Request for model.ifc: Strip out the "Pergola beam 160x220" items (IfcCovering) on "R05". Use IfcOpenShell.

First a look at what the model holds.

```python
import ifcopenshell
import ifcopenshell.util.element

model = ifcopenshell.open("model.ifc")
print(model.schema)
storey = next(s for s in model.by_type("IfcBuildingStorey") if s.Name == "R05")
coverings = [e for e in ifcopenshell.util.element.get_decomposition(storey) if e.is_a("IfcCovering")]
seen = {}
for e in coverings:
    element_type = ifcopenshell.util.element.get_type(e)
    name = element_type.Name if element_type not in (None, e) else None
    seen[name] = seen.get(name, 0) + 1
for name, count in sorted(seen.items(), key=str):
    print(count, "x", name)
```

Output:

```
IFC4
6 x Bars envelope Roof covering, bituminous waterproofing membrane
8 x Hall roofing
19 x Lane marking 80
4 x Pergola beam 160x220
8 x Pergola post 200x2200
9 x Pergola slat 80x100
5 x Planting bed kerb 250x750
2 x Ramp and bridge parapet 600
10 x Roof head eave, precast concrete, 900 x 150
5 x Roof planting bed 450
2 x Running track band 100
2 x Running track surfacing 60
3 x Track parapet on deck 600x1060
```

```python
import ifcopenshell
import ifcopenshell.api.root
import ifcopenshell.util.element

model = ifcopenshell.open("model.ifc")

storey = next(s for s in model.by_type("IfcBuildingStorey") if s.Name == "R05")
coverings = [e for e in ifcopenshell.util.element.get_decomposition(storey) if e.is_a("IfcCovering")]
targets = [e for e in coverings if (t := ifcopenshell.util.element.get_type(e)) not in (None, e) and t.Name == "Pergola beam 160x220"]

for e in targets:
    ifcopenshell.api.root.remove_product(model, product=e)
print(len(targets), "removed")

model.write("model_v2.ifc")
```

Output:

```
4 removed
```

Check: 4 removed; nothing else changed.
